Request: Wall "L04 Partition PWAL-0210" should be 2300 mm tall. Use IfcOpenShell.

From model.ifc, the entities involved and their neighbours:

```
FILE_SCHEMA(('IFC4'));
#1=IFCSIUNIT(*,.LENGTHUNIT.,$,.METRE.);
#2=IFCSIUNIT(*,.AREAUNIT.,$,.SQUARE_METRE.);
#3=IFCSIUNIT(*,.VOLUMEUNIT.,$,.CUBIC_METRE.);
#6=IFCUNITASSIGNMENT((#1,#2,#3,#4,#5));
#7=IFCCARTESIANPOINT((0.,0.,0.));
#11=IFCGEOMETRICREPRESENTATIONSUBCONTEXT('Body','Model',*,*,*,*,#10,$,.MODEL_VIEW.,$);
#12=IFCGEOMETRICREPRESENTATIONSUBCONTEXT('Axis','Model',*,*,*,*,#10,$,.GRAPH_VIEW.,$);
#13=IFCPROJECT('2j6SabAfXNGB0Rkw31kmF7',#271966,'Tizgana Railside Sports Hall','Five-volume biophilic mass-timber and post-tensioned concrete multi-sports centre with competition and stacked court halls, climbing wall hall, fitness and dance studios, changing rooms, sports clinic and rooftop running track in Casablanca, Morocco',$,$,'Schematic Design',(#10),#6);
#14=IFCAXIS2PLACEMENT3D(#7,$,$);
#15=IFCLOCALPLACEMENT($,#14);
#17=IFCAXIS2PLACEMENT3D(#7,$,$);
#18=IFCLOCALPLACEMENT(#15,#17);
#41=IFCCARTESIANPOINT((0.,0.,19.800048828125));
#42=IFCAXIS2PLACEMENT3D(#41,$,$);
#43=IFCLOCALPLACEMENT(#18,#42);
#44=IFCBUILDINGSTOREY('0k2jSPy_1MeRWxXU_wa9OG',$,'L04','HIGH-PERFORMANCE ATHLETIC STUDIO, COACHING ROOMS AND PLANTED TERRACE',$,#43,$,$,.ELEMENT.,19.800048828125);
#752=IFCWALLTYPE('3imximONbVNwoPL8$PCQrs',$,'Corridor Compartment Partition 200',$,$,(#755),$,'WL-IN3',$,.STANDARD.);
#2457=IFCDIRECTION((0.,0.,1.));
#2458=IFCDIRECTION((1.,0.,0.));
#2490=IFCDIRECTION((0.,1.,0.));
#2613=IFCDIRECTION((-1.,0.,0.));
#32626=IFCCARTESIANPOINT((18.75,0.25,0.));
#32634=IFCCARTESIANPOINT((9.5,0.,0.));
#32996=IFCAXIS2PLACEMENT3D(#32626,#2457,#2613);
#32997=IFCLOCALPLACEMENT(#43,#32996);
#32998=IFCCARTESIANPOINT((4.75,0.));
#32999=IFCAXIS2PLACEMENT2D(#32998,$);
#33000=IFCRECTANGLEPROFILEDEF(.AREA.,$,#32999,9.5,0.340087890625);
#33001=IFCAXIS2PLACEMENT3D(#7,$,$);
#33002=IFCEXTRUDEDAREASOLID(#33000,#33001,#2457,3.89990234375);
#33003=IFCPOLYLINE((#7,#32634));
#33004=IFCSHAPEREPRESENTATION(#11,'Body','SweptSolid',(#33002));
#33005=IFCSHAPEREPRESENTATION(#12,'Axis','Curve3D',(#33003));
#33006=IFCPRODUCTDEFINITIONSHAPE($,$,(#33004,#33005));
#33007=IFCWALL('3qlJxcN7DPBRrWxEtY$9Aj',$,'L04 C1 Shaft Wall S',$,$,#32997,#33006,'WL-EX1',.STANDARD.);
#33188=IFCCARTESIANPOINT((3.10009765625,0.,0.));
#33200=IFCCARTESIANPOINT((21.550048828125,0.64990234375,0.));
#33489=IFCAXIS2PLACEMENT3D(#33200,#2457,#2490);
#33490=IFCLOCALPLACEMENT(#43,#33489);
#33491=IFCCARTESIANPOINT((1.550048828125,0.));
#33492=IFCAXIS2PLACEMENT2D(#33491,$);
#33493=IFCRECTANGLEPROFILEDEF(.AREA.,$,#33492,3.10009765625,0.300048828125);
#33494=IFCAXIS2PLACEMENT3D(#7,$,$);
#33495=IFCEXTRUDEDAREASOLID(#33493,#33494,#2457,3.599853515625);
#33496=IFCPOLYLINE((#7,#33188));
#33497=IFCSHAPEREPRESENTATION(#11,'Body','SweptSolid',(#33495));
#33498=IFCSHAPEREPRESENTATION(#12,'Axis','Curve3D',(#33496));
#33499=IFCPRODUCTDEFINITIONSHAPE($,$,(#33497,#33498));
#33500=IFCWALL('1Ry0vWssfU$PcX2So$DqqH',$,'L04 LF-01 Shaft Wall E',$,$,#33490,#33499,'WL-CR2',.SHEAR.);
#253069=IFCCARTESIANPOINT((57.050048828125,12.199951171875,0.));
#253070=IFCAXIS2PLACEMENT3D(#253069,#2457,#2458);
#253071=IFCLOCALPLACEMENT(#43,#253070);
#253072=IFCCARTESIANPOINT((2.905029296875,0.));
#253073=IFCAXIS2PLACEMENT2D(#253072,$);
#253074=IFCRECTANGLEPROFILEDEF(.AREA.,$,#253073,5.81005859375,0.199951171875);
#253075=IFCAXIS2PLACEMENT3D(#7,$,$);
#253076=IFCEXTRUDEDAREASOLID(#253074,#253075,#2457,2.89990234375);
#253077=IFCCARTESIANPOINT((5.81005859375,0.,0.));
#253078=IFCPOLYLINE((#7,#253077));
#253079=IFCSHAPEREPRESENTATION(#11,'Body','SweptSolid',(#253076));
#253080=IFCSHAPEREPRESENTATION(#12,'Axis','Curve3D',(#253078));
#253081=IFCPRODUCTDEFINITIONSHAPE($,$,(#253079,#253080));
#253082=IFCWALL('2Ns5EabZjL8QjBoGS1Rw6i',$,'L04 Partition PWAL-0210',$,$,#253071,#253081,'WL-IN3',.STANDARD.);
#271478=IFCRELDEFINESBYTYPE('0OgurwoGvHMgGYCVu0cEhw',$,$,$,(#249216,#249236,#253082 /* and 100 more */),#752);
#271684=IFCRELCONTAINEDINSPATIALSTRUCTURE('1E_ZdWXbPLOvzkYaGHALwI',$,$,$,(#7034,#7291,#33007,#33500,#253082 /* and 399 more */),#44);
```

```python
import ifcopenshell
import ifcopenshell.geom
import ifcopenshell.util.representation
import ifcopenshell.util.shape
import ifcopenshell.util.unit

model = ifcopenshell.open("model.ifc")
unit_scale = ifcopenshell.util.unit.calculate_unit_scale(model)
settings = ifcopenshell.geom.settings()


def volume(element):
    """Net volume in cubic metres, openings subtracted."""
    shape = ifcopenshell.geom.create_shape(settings, element)
    return ifcopenshell.util.shape.get_volume(shape.geometry)


wall = model.by_guid("2Ns5EabZjL8QjBoGS1Rw6i")
before = volume(wall)

body = ifcopenshell.util.representation.get_representation(wall, "Model", "Body")
solid = body.Items[0]
old_height = solid.Depth
solid.Depth = 2.3 / unit_scale
after = volume(wall)

print(f"height {old_height:g} -> {solid.Depth:g}, volume {before:.3f} -> {after:.3f} m3")

model.write("model_updated.ifc")
```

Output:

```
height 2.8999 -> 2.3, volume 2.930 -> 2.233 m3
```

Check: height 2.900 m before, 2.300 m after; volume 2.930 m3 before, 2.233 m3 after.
